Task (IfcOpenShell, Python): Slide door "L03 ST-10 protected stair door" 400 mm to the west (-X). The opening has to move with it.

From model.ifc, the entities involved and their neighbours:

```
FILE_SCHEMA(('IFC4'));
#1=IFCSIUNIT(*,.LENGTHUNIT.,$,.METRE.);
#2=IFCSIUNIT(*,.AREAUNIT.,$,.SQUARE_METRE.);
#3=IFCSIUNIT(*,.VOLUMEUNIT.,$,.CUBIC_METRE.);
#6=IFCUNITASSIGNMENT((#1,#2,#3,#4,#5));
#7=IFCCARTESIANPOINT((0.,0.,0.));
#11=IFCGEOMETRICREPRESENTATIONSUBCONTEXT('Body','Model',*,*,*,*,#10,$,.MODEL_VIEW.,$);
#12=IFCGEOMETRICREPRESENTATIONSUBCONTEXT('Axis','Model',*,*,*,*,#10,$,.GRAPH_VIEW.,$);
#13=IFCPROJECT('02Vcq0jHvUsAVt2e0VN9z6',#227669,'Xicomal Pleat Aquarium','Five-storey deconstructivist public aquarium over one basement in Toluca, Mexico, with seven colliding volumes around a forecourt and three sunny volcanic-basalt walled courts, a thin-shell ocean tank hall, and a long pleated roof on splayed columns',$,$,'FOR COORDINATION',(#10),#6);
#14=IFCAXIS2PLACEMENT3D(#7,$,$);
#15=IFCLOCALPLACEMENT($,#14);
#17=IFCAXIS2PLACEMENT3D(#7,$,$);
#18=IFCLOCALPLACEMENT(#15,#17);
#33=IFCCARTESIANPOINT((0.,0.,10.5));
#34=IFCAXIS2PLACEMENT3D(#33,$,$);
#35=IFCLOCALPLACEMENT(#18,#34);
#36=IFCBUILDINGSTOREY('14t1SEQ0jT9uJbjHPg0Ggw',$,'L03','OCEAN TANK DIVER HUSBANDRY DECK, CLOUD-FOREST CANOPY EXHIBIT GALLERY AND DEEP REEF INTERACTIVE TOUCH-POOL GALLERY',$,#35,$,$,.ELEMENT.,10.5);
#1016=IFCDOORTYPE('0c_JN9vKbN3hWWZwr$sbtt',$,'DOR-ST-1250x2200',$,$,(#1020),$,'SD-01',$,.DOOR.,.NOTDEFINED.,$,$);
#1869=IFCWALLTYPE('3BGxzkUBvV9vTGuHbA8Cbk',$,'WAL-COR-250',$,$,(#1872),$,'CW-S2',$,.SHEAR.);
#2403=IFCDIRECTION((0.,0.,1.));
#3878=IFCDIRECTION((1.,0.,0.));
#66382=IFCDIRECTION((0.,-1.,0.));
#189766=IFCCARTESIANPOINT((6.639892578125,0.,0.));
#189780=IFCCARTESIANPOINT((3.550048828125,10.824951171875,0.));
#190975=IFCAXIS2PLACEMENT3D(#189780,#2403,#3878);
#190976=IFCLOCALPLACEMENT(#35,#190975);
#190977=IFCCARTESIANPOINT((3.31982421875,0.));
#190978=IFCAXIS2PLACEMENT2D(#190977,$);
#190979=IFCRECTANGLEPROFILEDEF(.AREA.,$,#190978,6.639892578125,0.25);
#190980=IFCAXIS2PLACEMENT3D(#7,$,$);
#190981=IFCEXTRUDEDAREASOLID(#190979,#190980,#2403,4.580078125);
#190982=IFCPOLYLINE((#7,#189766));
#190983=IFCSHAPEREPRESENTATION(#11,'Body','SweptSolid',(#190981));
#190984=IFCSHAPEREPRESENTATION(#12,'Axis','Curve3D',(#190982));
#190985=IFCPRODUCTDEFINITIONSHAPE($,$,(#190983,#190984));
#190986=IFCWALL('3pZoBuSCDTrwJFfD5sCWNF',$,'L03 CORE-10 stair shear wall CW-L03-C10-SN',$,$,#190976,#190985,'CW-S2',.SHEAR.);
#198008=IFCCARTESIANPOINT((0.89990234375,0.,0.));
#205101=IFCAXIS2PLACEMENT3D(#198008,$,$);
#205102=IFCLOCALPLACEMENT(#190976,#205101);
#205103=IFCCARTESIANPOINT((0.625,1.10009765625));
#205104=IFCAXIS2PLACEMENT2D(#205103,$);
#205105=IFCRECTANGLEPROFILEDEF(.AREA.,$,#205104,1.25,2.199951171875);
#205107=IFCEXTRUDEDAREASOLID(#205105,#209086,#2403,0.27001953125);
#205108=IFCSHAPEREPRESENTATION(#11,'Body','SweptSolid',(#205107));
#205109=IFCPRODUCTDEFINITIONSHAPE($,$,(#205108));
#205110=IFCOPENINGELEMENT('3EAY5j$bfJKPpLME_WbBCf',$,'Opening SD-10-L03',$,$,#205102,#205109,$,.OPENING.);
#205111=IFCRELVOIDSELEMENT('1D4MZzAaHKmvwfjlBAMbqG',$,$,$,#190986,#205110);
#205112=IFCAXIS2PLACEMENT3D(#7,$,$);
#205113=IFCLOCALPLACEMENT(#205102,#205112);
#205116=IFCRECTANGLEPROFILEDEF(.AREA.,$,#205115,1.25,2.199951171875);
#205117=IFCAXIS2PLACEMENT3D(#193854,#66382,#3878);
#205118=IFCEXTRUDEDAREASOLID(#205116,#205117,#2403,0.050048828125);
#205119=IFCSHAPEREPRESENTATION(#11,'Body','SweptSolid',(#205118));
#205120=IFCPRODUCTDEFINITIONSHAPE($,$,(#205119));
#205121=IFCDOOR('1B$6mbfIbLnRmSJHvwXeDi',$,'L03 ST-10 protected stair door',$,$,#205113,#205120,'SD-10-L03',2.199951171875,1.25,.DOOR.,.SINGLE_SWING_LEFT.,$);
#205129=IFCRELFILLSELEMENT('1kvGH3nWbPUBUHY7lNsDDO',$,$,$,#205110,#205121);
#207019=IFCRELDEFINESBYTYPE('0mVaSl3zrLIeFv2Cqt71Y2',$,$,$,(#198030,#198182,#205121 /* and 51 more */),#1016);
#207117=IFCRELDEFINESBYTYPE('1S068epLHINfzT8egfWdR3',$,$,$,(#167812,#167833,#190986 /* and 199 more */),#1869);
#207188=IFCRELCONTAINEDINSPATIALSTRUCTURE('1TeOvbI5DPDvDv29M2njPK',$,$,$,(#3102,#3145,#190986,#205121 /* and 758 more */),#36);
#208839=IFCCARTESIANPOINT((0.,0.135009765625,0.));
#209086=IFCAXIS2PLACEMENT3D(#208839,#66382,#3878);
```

```python
import ifcopenshell
import ifcopenshell.api.geometry
import ifcopenshell.util.placement

model = ifcopenshell.open("model.ifc")

door = model.by_guid("1B$6mbfIbLnRmSJHvwXeDi")
opening = door.FillsVoids[0].RelatingOpeningElement
wall = opening.VoidsElements[0].RelatingBuildingElement

wall_matrix = ifcopenshell.util.placement.get_local_placement(wall.ObjectPlacement)
shift = wall_matrix[:3, 0] * -0.4
before = ifcopenshell.util.placement.get_local_placement(door.ObjectPlacement)[:3, 3].copy()

# The door is placed relative to its opening, so it follows when the opening moves.
matrix = ifcopenshell.util.placement.get_local_placement(opening.ObjectPlacement)
matrix[:3, 3] += shift
ifcopenshell.api.geometry.edit_object_placement(
    model, product=opening, matrix=matrix, is_si=False, should_transform_children=True
)

after = ifcopenshell.util.placement.get_local_placement(door.ObjectPlacement)[:3, 3]
print("door moved by", (after - before).round(3) + 0.0)

model.write("model_updated.ifc")
```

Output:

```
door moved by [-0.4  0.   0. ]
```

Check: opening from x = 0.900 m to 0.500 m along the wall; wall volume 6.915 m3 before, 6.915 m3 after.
